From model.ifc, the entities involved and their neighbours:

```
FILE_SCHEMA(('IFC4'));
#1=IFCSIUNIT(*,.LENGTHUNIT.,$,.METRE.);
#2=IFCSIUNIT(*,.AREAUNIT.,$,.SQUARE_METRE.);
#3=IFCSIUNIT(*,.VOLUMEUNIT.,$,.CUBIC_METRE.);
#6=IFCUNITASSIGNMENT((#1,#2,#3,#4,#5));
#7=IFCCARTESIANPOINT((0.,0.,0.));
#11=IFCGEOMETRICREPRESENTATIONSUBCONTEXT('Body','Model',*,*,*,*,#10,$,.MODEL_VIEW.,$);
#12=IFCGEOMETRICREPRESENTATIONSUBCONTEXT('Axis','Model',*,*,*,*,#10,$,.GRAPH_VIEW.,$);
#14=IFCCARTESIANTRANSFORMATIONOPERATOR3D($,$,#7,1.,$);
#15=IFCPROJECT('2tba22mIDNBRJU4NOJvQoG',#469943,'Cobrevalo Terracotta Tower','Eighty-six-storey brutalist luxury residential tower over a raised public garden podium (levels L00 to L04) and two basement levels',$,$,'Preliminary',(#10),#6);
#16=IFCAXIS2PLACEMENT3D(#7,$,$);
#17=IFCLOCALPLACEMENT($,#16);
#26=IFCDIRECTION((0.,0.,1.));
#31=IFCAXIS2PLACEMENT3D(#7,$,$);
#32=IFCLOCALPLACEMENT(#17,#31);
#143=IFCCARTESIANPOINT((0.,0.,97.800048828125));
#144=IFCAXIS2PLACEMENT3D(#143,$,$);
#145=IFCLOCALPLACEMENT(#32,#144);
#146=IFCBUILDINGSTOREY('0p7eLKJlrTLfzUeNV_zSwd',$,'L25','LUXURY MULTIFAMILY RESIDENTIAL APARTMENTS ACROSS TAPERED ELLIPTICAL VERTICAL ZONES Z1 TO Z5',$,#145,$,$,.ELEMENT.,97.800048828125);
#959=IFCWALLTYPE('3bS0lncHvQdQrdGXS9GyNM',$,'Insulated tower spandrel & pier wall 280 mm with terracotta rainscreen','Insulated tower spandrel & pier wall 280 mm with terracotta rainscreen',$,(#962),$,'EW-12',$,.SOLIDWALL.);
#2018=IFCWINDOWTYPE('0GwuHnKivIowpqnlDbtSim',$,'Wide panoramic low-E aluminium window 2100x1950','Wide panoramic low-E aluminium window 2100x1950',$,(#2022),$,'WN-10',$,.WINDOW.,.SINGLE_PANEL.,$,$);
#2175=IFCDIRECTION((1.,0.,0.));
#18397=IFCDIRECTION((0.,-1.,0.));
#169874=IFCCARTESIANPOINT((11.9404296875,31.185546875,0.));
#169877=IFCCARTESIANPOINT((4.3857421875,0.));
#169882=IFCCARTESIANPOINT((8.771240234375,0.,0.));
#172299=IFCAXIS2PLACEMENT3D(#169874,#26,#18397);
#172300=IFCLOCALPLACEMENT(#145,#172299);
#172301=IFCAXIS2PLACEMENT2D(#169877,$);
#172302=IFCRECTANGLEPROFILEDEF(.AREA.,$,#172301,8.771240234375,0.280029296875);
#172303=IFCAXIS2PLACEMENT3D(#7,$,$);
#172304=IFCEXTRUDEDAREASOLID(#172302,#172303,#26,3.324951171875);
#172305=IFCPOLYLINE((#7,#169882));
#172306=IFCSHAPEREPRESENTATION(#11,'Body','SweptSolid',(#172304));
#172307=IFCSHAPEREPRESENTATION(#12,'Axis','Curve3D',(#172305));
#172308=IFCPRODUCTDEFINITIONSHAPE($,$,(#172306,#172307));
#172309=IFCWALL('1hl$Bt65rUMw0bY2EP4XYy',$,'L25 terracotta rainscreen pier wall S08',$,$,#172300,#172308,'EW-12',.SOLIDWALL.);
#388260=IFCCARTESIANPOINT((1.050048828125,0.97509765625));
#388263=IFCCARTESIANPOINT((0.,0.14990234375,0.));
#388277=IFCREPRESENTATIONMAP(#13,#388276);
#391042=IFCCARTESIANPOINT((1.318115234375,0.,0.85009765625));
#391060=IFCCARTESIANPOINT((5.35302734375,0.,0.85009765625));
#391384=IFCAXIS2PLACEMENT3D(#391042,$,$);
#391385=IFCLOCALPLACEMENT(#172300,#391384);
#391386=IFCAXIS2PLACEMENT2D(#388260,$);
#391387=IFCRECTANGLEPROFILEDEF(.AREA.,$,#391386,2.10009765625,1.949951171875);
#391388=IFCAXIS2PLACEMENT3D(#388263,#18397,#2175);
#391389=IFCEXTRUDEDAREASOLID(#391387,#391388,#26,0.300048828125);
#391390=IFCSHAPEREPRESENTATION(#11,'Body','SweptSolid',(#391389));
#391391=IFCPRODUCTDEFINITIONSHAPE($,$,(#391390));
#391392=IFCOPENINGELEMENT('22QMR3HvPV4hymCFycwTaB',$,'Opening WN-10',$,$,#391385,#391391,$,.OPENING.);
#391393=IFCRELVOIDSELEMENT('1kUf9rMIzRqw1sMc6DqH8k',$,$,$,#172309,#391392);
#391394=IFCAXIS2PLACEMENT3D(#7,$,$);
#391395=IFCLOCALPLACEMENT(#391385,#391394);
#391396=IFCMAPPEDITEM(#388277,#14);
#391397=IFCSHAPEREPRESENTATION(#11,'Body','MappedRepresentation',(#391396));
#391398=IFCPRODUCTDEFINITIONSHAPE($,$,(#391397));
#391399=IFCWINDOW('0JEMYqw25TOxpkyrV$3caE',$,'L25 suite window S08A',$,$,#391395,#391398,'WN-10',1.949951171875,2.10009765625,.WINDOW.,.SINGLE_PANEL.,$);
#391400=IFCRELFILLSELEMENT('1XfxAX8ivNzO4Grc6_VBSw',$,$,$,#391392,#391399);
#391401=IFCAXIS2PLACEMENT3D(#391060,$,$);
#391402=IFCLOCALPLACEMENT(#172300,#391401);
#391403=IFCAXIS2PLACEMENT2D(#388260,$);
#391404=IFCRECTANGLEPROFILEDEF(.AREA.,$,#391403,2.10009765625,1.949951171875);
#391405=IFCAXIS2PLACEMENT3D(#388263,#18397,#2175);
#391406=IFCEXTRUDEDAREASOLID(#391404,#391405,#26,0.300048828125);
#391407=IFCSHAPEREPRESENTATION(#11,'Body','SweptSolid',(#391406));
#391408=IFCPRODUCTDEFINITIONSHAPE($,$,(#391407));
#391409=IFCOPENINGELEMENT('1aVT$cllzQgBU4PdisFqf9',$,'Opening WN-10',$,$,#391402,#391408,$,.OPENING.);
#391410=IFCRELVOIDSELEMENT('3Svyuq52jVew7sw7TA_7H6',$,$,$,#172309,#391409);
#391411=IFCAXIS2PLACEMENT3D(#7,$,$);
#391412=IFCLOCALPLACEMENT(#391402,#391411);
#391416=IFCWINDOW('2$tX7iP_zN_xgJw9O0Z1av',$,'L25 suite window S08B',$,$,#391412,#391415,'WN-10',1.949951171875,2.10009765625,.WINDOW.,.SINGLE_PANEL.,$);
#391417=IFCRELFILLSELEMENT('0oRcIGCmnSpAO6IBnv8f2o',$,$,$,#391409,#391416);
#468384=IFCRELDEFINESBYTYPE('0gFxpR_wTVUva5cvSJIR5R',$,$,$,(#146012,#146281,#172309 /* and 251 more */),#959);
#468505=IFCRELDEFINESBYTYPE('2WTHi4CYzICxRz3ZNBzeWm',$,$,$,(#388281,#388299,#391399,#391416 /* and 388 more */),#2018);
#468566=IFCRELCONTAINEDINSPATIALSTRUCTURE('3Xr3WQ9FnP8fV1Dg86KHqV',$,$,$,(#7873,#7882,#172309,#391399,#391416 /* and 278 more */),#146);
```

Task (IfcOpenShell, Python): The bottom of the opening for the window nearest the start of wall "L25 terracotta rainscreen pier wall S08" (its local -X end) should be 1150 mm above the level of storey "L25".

```python
import numpy as np
import ifcopenshell
import ifcopenshell.api.geometry
import ifcopenshell.geom
import ifcopenshell.util.element
import ifcopenshell.util.placement
import ifcopenshell.util.shape
import ifcopenshell.util.unit

model = ifcopenshell.open("model.ifc")
unit_scale = ifcopenshell.util.unit.calculate_unit_scale(model)

window = model.by_guid("0JEMYqw25TOxpkyrV$3caE")
opening = window.FillsVoids[0].RelatingOpeningElement
storey = ifcopenshell.util.element.get_container(window, ifc_class="IfcBuildingStorey")
level = ifcopenshell.util.placement.get_local_placement(storey.ObjectPlacement)[2, 3]

# The opening's origin need not be at the sill, so measure its lowest point.
shape = ifcopenshell.geom.create_shape(ifcopenshell.geom.settings(), opening)
bottom = ifcopenshell.util.shape.get_shape_bottom_elevation(shape, shape.geometry) / unit_scale
dz = level + 1.15 - bottom

shift = np.array([0.0, 0.0, dz])
# The window is placed relative to its opening, so it follows when the opening moves.
matrix = ifcopenshell.util.placement.get_local_placement(opening.ObjectPlacement)
matrix[:3, 3] += shift
ifcopenshell.api.geometry.edit_object_placement(
    model, product=opening, matrix=matrix, is_si=False, should_transform_children=True
)

print(f"moved by {dz * unit_scale:+.3f} m")

model.write("model_v2.ifc")
```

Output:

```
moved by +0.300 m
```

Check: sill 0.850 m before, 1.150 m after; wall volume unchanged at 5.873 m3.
